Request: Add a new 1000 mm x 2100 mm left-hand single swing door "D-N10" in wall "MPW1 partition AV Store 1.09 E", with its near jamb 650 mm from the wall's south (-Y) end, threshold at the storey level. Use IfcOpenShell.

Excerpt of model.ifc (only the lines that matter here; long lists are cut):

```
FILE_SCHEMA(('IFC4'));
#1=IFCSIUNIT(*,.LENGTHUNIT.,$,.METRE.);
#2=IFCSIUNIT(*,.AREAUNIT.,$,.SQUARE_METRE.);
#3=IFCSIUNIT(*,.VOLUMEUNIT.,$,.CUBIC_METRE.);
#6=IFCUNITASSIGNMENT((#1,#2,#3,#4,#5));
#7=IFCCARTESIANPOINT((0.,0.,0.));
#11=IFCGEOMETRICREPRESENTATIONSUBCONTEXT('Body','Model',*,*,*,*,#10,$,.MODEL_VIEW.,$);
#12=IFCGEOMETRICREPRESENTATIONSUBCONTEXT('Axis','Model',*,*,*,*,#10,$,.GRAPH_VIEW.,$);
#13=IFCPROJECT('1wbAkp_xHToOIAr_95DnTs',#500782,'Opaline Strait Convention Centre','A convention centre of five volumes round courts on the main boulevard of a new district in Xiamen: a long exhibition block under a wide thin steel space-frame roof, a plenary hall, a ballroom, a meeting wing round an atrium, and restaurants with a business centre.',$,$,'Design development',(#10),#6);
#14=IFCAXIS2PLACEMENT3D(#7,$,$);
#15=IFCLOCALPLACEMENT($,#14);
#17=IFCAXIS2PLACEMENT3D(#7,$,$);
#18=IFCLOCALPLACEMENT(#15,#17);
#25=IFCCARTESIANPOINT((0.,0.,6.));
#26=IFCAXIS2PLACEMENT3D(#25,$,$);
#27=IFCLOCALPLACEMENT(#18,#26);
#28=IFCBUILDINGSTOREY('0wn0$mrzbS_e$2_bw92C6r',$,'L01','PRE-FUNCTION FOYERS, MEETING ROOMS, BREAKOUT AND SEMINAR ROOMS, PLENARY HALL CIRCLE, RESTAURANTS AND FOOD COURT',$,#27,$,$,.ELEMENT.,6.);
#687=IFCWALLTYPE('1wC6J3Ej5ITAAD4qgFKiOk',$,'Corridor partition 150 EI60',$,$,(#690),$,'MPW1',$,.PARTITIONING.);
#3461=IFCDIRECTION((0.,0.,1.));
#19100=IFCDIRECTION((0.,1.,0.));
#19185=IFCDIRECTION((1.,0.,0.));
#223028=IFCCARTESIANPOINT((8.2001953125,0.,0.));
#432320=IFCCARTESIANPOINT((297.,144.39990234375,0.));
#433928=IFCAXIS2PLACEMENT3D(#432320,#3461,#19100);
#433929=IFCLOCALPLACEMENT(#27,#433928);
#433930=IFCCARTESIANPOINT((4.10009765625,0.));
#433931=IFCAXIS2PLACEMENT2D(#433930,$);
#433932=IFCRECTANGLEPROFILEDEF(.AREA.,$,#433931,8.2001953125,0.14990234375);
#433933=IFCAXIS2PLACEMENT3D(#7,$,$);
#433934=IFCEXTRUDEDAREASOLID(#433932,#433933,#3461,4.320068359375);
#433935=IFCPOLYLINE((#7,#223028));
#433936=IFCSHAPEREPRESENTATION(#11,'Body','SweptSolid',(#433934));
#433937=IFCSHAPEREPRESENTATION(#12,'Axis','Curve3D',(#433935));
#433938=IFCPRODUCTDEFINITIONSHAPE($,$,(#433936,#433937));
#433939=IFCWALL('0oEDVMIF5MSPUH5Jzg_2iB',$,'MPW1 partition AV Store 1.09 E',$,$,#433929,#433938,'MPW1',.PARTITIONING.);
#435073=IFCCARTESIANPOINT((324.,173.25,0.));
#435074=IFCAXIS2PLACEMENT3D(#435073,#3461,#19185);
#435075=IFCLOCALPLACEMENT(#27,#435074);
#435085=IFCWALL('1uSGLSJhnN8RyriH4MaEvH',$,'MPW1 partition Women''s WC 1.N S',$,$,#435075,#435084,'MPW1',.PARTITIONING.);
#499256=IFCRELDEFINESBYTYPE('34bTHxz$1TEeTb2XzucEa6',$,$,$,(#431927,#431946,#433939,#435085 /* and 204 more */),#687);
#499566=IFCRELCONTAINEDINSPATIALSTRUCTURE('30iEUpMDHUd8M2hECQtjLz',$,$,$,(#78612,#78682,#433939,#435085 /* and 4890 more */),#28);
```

```python
import numpy as np
import ifcopenshell
import ifcopenshell.api.feature
import ifcopenshell.api.geometry
import ifcopenshell.api.root
import ifcopenshell.api.spatial
import ifcopenshell.geom
import ifcopenshell.util.element
import ifcopenshell.util.placement
import ifcopenshell.util.representation
import ifcopenshell.util.shape
import ifcopenshell.util.unit

model = ifcopenshell.open("model.ifc")
unit_scale = ifcopenshell.util.unit.calculate_unit_scale(model)
settings = ifcopenshell.geom.settings()


def volume(element):
    """Net volume in cubic metres, openings subtracted."""
    shape = ifcopenshell.geom.create_shape(settings, element)
    return ifcopenshell.util.shape.get_volume(shape.geometry)


wall = model.by_guid("0oEDVMIF5MSPUH5Jzg_2iB")
storey = ifcopenshell.util.element.get_container(wall, ifc_class="IfcBuildingStorey")
context = ifcopenshell.util.representation.get_context(model, "Model", "Body", "MODEL_VIEW")
before = volume(wall)

width, height, from_end, sill = 1, 2.1, 0.65, 0.0  # metres

# The wall runs along its own X axis, and the end named is its -X end.
wall_shape = ifcopenshell.geom.create_shape(settings, wall)
x, y, z = ifcopenshell.util.shape.get_vertices(wall_shape.geometry).T
start = x.min() + from_end
face, thickness = float(y.min()), float(y.max() - y.min())
wall_matrix = ifcopenshell.util.placement.get_local_placement(wall.ObjectPlacement)
level = ifcopenshell.util.placement.get_local_placement(storey.ObjectPlacement)[2, 3]


def in_wall(x, y):
    """Placement at x, y metres in the wall's axes, at sill height."""
    matrix = wall_matrix.copy()
    matrix[:, 3] = wall_matrix @ np.array([x / unit_scale, y / unit_scale, 0.0, 1.0])
    matrix[2, 3] = level + sill / unit_scale
    return matrix


# Opening: a box that overshoots both wall faces by 50 mm.
opening = ifcopenshell.api.root.create_entity(model, ifc_class="IfcOpeningElement", predefined_type="OPENING")
box = ifcopenshell.api.geometry.add_wall_representation(
    model, context=context, length=width, height=height, thickness=thickness + 0.1
)
ifcopenshell.api.geometry.assign_representation(model, product=opening, representation=box)
ifcopenshell.api.geometry.edit_object_placement(model, product=opening, matrix=in_wall(start, face - 0.05), is_si=False)
ifcopenshell.api.feature.add_feature(model, feature=opening, element=wall)

door = ifcopenshell.api.root.create_entity(model, ifc_class="IfcDoor", name="D-N10", predefined_type="DOOR")
door.OverallWidth, door.OverallHeight = width / unit_scale, height / unit_scale
door.OperationType = "SINGLE_SWING_LEFT"
body = ifcopenshell.api.geometry.add_door_representation(
    model,
    context=context,
    overall_width=door.OverallWidth,
    overall_height=door.OverallHeight,
    operation_type="SINGLE_SWING_LEFT",
    lining_properties={"LiningDepth": thickness / unit_scale, "ThresholdDepth": thickness / unit_scale},
)
ifcopenshell.api.geometry.assign_representation(model, product=door, representation=body)
ifcopenshell.api.spatial.assign_container(model, products=[door], relating_structure=storey)
ifcopenshell.api.feature.add_filling(model, opening=opening, element=door)

# The lining spans the wall, so the door starts at the wall face.
ifcopenshell.api.geometry.edit_object_placement(model, product=door, matrix=in_wall(start, face), is_si=False)

after = volume(wall)

print(f"wall volume {before:.3f} -> {after:.3f} m3")

model.write("model_rev.ifc")
```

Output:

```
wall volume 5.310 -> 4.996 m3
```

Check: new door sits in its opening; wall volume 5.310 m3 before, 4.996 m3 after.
